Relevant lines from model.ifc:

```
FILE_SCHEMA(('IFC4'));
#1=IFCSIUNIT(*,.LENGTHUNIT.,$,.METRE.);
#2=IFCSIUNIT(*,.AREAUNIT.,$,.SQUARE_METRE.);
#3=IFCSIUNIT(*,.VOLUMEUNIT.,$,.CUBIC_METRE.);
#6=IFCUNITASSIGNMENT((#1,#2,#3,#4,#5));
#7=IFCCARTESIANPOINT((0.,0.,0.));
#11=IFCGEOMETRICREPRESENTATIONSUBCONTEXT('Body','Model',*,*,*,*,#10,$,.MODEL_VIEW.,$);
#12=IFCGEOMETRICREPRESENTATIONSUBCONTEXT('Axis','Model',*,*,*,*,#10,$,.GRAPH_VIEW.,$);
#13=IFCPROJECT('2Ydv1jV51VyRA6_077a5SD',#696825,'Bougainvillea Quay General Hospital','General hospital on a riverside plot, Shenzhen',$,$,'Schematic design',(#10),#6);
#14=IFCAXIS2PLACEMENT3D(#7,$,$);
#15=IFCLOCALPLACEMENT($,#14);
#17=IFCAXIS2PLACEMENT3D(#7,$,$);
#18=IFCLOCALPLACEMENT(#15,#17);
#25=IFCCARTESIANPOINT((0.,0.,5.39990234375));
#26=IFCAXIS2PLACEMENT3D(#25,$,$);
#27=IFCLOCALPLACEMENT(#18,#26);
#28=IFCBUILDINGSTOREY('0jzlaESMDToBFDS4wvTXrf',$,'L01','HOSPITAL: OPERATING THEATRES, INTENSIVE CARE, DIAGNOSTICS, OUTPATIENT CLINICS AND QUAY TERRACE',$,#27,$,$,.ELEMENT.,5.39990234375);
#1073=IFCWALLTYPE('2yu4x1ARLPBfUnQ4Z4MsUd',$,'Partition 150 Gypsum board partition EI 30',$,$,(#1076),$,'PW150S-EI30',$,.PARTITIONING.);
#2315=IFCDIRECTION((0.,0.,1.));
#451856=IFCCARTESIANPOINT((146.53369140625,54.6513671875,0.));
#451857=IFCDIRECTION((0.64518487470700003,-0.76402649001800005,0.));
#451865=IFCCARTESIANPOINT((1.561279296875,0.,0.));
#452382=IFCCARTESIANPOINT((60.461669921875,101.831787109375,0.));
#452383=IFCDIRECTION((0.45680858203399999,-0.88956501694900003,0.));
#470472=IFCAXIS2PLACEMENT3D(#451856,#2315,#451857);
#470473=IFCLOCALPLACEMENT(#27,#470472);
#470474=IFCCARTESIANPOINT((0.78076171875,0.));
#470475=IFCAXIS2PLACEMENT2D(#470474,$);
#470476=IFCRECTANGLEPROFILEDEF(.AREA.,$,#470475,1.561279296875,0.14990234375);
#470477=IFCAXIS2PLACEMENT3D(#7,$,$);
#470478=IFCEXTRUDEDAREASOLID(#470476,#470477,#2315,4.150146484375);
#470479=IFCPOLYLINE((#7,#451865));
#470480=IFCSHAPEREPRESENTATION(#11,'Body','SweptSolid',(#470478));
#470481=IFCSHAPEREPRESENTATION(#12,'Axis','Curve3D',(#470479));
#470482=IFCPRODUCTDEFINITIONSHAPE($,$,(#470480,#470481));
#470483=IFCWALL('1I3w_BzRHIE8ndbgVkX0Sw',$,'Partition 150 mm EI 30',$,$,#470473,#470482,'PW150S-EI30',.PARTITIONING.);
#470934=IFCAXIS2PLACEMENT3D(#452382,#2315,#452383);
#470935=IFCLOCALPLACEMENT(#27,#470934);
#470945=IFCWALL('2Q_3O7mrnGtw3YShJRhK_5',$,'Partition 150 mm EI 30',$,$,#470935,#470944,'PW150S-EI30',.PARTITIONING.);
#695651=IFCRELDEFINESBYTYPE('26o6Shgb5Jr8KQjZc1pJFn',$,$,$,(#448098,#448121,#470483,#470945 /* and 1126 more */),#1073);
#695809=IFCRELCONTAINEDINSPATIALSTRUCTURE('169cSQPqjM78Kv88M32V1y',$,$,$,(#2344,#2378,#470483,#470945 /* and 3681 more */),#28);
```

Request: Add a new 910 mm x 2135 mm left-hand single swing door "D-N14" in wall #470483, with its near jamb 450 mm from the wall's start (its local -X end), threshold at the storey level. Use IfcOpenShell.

```python
import numpy as np
import ifcopenshell
import ifcopenshell.api.feature
import ifcopenshell.api.geometry
import ifcopenshell.api.root
import ifcopenshell.api.spatial
import ifcopenshell.geom
import ifcopenshell.util.element
import ifcopenshell.util.placement
import ifcopenshell.util.representation
import ifcopenshell.util.shape
import ifcopenshell.util.unit

model = ifcopenshell.open("model.ifc")
unit_scale = ifcopenshell.util.unit.calculate_unit_scale(model)
settings = ifcopenshell.geom.settings()


def volume(element):
    """Net volume in cubic metres, openings subtracted."""
    shape = ifcopenshell.geom.create_shape(settings, element)
    return ifcopenshell.util.shape.get_volume(shape.geometry)


wall = model.by_guid("1I3w_BzRHIE8ndbgVkX0Sw")
storey = ifcopenshell.util.element.get_container(wall, ifc_class="IfcBuildingStorey")
context = ifcopenshell.util.representation.get_context(model, "Model", "Body", "MODEL_VIEW")
before = volume(wall)

width, height, from_end, sill = 0.91, 2.135, 0.45, 0.0  # metres

# The wall runs along its own X axis, and the end named is its -X end.
wall_shape = ifcopenshell.geom.create_shape(settings, wall)
x, y, z = ifcopenshell.util.shape.get_vertices(wall_shape.geometry).T
start = x.min() + from_end
face, thickness = float(y.min()), float(y.max() - y.min())
wall_matrix = ifcopenshell.util.placement.get_local_placement(wall.ObjectPlacement)
level = ifcopenshell.util.placement.get_local_placement(storey.ObjectPlacement)[2, 3]


def in_wall(x, y):
    """Placement at x, y metres in the wall's axes, at sill height."""
    matrix = wall_matrix.copy()
    matrix[:, 3] = wall_matrix @ np.array([x / unit_scale, y / unit_scale, 0.0, 1.0])
    matrix[2, 3] = level + sill / unit_scale
    return matrix


# Opening: a box that overshoots both wall faces by 50 mm.
opening = ifcopenshell.api.root.create_entity(model, ifc_class="IfcOpeningElement", predefined_type="OPENING")
box = ifcopenshell.api.geometry.add_wall_representation(
    model, context=context, length=width, height=height, thickness=thickness + 0.1
)
ifcopenshell.api.geometry.assign_representation(model, product=opening, representation=box)
ifcopenshell.api.geometry.edit_object_placement(model, product=opening, matrix=in_wall(start, face - 0.05), is_si=False)
ifcopenshell.api.feature.add_feature(model, feature=opening, element=wall)

door = ifcopenshell.api.root.create_entity(model, ifc_class="IfcDoor", name="D-N14", predefined_type="DOOR")
door.OverallWidth, door.OverallHeight = width / unit_scale, height / unit_scale
door.OperationType = "SINGLE_SWING_LEFT"
body = ifcopenshell.api.geometry.add_door_representation(
    model,
    context=context,
    overall_width=door.OverallWidth,
    overall_height=door.OverallHeight,
    operation_type="SINGLE_SWING_LEFT",
    lining_properties={"LiningDepth": thickness / unit_scale, "ThresholdDepth": thickness / unit_scale},
)
ifcopenshell.api.geometry.assign_representation(model, product=door, representation=body)
ifcopenshell.api.spatial.assign_container(model, products=[door], relating_structure=storey)
ifcopenshell.api.feature.add_filling(model, opening=opening, element=door)

# The lining spans the wall, so the door starts at the wall face.
ifcopenshell.api.geometry.edit_object_placement(model, product=door, matrix=in_wall(start, face), is_si=False)

after = volume(wall)

print(f"wall volume {before:.3f} -> {after:.3f} m3")

model.write("model_updated.ifc")
```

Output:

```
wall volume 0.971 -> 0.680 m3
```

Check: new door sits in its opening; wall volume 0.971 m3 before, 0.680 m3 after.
